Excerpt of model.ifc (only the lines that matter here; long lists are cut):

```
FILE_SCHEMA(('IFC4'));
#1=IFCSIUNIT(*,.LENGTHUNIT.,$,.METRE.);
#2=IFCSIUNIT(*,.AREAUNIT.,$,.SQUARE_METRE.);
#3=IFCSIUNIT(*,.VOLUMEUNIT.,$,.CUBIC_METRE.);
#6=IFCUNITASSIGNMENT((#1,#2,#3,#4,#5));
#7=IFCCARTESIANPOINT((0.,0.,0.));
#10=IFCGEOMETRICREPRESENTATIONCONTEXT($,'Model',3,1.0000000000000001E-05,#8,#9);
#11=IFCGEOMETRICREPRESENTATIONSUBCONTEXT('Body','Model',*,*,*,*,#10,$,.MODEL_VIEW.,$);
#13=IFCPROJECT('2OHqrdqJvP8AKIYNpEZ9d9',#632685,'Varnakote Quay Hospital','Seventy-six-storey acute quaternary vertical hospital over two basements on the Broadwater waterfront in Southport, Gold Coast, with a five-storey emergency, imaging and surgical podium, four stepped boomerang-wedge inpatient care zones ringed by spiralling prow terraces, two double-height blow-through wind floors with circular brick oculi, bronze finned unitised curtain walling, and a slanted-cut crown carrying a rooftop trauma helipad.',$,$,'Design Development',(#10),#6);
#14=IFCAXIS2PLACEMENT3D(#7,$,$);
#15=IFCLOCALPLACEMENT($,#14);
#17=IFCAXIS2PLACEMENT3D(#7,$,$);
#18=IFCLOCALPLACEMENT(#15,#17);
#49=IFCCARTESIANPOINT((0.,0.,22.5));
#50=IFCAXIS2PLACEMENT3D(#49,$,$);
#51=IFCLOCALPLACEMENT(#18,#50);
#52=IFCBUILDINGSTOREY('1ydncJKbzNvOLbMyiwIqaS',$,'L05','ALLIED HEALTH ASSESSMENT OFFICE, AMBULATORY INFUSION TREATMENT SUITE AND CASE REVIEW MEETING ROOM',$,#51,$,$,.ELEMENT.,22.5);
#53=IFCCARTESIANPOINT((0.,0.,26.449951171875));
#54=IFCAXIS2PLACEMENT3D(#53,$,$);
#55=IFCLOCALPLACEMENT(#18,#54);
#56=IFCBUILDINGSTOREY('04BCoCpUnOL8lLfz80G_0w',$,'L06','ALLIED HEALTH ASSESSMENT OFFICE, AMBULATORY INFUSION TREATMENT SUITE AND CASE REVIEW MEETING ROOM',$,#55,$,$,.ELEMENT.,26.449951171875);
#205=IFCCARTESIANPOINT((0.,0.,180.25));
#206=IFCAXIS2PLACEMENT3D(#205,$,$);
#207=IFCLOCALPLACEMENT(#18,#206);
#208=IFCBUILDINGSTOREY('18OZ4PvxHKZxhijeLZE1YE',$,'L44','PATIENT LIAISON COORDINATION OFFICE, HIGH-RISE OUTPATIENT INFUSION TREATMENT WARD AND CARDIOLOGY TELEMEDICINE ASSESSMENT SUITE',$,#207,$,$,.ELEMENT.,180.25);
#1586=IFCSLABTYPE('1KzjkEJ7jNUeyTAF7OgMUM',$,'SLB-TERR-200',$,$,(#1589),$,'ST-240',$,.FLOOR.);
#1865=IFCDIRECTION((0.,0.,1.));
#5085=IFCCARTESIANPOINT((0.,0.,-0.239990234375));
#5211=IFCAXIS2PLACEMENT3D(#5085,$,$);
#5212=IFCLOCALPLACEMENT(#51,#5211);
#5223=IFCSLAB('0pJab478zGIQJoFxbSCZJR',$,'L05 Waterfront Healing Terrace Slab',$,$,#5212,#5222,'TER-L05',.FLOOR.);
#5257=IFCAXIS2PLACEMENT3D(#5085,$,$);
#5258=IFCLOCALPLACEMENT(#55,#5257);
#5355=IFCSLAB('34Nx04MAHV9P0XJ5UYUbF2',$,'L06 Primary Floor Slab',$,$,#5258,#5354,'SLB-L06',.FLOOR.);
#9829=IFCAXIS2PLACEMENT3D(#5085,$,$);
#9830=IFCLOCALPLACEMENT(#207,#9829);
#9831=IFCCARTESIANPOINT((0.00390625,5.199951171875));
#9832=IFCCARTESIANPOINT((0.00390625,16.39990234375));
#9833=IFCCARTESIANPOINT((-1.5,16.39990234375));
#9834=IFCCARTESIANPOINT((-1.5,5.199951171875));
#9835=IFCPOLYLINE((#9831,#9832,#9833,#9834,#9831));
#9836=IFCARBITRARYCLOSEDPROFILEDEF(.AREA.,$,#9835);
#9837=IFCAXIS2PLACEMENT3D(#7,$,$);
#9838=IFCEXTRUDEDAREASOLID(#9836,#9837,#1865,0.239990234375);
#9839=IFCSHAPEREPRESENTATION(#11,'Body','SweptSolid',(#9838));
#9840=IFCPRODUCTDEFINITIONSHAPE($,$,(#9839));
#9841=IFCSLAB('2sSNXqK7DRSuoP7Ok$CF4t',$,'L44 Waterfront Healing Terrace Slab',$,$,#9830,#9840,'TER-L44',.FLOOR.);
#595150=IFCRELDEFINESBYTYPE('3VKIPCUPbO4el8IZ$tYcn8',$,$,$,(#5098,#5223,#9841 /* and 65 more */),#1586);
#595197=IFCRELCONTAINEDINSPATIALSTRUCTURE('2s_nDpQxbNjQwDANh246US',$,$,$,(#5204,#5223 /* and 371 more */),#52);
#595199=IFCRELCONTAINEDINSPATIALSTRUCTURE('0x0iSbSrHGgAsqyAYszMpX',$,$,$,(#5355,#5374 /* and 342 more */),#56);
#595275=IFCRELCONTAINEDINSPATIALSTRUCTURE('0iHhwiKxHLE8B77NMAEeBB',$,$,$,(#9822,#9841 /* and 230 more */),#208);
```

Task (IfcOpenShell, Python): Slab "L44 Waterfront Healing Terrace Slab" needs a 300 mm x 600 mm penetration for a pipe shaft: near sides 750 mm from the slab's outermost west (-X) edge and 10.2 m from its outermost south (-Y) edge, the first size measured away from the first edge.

```python
import numpy as np
import ifcopenshell
import ifcopenshell.api.feature
import ifcopenshell.api.geometry
import ifcopenshell.api.root
import ifcopenshell.geom
import ifcopenshell.util.placement
import ifcopenshell.util.representation
import ifcopenshell.util.shape
import ifcopenshell.util.unit

model = ifcopenshell.open("model.ifc")
unit_scale = ifcopenshell.util.unit.calculate_unit_scale(model)
settings = ifcopenshell.geom.settings()


def volume(element):
    """Net volume in cubic metres, openings subtracted."""
    shape = ifcopenshell.geom.create_shape(settings, element)
    return ifcopenshell.util.shape.get_volume(shape.geometry)


slab = model.by_id(9841)
before = volume(slab)

# Extent in the slab's own axes, in metres. The edges named are its -X and -Y sides.
slab_shape = ifcopenshell.geom.create_shape(settings, slab)
vertices = ifcopenshell.util.shape.get_vertices(slab_shape.geometry)
x_min, y_min, bottom = vertices.min(axis=0)
top = vertices[:, 2].max()

opening = ifcopenshell.api.root.create_entity(model, ifc_class="IfcOpeningElement", name="Pipe shaft opening", predefined_type="OPENING")
context = ifcopenshell.util.representation.get_context(model, "Model", "Body", "MODEL_VIEW")
width, depth = 0.3, 0.6
outline = [(0.0, 0.0), (width, 0.0), (width, depth), (0.0, depth), (0.0, 0.0)]
# Overshoot both faces by 50 mm so the cut is clean.
shape = ifcopenshell.api.geometry.add_slab_representation(
    model, context=context, depth=top - bottom + 0.1, polyline=outline
)
ifcopenshell.api.geometry.assign_representation(model, product=opening, representation=shape)

matrix = ifcopenshell.util.placement.get_local_placement(slab.ObjectPlacement)
matrix[:, 3] = matrix @ np.append(np.array([x_min + 0.75, y_min + 10.2, bottom - 0.05]) / unit_scale, 1.0)
ifcopenshell.api.geometry.edit_object_placement(model, product=opening, matrix=matrix, is_si=False)
ifcopenshell.api.feature.add_feature(model, feature=opening, element=slab)

after = volume(slab)

print(f"slab volume {before:.3f} -> {after:.3f} m3")

model.write("model_rev.ifc")
```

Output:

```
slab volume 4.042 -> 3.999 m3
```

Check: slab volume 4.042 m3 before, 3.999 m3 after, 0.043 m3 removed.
